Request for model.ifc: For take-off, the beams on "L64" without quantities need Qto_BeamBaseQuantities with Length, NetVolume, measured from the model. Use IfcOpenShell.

First a look at what the model holds.

```python
import ifcopenshell
import ifcopenshell.util.element
import ifcopenshell.util.unit

model = ifcopenshell.open("model.ifc")
print(model.schema)
for unit_type in ("LENGTHUNIT", "AREAUNIT", "VOLUMEUNIT"):
    print(unit_type, ifcopenshell.util.unit.calculate_unit_scale(model, unit_type))
storey = next(s for s in model.by_type("IfcBuildingStorey") if s.Name == "L64")
beams = [e for e in ifcopenshell.util.element.get_decomposition(storey) if e.is_a("IfcBeam")]
for e in sorted(beams, key=lambda e: e.id()):
    print(e.id(), e.is_a(), e.Name, list(ifcopenshell.util.element.get_psets(e, qtos_only=True)), sep=" | ")
```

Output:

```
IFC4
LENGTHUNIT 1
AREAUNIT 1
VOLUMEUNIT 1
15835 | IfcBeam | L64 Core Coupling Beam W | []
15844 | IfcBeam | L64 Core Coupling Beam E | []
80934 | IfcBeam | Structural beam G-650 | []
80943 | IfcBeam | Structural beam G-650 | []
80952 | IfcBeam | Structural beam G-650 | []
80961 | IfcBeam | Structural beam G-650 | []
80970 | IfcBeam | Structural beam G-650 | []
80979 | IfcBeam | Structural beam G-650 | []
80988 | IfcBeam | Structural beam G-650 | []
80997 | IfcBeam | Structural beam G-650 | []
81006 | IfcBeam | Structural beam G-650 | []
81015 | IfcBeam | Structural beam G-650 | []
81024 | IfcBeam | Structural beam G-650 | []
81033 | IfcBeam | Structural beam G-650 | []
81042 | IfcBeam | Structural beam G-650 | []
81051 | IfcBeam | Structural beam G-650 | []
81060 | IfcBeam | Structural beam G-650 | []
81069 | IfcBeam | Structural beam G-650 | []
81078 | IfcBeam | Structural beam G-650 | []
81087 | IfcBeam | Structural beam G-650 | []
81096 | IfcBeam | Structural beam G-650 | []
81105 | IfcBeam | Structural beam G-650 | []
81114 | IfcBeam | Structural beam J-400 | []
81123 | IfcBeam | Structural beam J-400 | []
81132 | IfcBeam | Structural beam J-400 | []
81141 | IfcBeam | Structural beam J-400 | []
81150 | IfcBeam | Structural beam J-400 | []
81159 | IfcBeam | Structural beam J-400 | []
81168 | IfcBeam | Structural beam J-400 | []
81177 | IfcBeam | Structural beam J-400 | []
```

```python
import ifcopenshell
import ifcopenshell.api.pset
import ifcopenshell.geom
import ifcopenshell.util.element
import ifcopenshell.util.shape
import ifcopenshell.util.unit

model = ifcopenshell.open("model.ifc")
unit_scale = ifcopenshell.util.unit.calculate_unit_scale(model)
volume_scale = ifcopenshell.util.unit.calculate_unit_scale(model, "VOLUMEUNIT")
settings = ifcopenshell.geom.settings()

storey = next(s for s in model.by_type("IfcBuildingStorey") if s.Name == "L64")
beams = [e for e in ifcopenshell.util.element.get_decomposition(storey) if e.is_a("IfcBeam")]

for e in sorted(beams, key=lambda e: e.id()):
    if ifcopenshell.util.element.get_psets(e, qtos_only=True, should_inherit=False):
        continue
    # Geometry comes back in metres, in the element's own axes.
    shape = ifcopenshell.geom.create_shape(settings, e)
    values = {
        "Length": ifcopenshell.util.shape.get_max_xyz(shape.geometry) / unit_scale,
        "NetVolume": ifcopenshell.util.shape.get_volume(shape.geometry) / volume_scale,
    }
    qto = ifcopenshell.api.pset.add_qto(model, product=e, name="Qto_BeamBaseQuantities")
    ifcopenshell.api.pset.edit_qto(model, qto=qto, properties=values)
    print(e.id(), {k: round(v, 3) for k, v in values.items()})

model.write("model_v2.ifc")
```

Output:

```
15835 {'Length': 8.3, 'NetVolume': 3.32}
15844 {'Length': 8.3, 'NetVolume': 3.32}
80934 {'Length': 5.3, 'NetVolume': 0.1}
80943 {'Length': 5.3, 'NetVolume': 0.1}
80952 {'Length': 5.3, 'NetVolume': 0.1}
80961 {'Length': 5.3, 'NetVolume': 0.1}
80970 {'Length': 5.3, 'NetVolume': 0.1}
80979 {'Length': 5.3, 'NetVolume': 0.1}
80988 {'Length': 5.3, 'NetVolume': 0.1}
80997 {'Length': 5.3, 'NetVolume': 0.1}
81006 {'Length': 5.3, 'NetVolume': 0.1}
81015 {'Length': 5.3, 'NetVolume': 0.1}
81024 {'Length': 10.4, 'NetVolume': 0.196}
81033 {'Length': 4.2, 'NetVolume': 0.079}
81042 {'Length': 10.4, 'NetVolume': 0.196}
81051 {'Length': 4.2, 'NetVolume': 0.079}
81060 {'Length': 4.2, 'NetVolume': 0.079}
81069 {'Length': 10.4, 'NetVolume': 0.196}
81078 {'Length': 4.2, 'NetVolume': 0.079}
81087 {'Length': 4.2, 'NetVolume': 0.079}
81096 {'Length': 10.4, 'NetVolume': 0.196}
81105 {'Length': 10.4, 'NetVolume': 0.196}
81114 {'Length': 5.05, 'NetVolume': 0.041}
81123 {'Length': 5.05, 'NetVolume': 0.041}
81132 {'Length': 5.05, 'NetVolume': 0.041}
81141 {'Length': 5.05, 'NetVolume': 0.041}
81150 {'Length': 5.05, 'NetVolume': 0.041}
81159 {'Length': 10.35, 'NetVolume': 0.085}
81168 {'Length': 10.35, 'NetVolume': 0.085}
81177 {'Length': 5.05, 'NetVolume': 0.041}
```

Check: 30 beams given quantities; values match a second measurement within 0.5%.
